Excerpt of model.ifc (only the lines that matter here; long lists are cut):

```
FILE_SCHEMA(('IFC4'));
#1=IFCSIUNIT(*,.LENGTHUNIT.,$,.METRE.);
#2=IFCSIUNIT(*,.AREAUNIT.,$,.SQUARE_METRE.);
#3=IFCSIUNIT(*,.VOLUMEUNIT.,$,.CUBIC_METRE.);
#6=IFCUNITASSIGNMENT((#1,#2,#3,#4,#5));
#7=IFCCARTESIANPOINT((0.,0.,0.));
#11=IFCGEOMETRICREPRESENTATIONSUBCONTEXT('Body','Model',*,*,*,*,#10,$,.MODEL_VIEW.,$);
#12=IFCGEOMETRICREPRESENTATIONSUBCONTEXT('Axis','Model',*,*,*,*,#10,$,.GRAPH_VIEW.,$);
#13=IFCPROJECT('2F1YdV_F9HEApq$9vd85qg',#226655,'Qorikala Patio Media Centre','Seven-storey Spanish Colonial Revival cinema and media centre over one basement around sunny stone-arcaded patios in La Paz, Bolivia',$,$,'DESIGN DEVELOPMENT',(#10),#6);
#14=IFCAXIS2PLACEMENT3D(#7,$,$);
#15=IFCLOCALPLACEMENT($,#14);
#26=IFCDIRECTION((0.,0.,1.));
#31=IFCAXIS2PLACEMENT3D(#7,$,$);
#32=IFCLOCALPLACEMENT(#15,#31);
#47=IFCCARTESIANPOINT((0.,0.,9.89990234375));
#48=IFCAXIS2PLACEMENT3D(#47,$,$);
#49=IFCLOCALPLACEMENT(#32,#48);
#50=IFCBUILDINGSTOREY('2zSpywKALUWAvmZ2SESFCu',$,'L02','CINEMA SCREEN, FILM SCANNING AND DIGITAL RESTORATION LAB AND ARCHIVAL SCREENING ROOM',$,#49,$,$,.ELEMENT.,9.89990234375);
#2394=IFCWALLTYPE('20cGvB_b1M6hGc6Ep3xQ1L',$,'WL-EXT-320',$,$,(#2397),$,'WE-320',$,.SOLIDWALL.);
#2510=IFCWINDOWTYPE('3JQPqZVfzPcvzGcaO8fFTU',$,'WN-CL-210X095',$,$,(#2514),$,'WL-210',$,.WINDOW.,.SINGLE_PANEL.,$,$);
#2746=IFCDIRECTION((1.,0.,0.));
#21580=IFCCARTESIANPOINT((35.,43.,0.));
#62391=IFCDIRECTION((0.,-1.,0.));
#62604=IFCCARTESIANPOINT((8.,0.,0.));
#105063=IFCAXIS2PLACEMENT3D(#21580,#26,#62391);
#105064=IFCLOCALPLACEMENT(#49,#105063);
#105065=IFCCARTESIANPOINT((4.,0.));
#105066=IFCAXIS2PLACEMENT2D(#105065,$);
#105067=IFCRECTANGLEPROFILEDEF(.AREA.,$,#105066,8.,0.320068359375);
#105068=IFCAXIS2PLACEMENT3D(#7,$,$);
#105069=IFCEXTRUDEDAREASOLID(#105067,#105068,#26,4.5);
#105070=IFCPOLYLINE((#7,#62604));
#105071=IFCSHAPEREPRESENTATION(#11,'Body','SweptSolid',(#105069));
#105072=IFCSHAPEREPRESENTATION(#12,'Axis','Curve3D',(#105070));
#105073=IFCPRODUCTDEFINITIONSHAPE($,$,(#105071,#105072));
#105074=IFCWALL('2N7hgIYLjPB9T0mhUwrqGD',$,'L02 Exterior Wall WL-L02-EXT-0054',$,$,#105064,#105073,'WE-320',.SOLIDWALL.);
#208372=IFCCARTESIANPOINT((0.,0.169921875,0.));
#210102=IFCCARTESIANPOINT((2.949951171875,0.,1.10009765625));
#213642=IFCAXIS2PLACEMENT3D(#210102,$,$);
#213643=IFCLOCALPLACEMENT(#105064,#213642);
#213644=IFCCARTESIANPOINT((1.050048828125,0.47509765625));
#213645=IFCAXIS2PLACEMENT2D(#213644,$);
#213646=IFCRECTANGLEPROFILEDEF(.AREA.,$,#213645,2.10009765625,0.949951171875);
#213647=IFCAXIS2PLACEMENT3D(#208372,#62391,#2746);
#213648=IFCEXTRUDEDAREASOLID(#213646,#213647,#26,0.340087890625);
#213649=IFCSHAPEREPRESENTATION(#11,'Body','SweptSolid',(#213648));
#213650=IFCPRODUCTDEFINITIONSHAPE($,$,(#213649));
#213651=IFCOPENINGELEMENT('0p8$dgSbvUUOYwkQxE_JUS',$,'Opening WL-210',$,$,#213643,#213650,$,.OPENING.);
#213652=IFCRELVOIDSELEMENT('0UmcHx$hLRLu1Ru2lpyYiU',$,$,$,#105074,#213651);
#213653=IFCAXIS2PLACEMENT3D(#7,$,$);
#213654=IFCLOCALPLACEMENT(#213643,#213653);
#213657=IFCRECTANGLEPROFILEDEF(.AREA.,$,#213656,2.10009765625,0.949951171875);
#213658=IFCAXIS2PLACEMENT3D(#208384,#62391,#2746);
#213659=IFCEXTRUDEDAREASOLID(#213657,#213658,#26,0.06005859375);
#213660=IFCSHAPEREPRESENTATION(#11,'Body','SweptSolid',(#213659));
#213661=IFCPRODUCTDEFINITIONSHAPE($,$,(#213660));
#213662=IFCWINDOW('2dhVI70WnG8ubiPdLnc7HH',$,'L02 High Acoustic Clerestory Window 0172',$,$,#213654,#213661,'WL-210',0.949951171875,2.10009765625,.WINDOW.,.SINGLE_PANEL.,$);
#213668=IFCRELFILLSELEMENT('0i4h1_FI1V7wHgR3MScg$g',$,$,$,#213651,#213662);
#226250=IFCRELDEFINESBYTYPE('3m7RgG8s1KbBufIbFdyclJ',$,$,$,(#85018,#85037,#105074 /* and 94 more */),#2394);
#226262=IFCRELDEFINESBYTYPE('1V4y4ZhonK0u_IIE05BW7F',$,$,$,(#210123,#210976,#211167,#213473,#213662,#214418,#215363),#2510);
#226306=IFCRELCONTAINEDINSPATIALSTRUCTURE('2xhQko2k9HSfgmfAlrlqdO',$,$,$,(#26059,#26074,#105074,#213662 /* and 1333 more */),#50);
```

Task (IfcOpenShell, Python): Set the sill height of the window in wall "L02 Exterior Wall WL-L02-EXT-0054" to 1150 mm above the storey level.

```python
import numpy as np
import ifcopenshell
import ifcopenshell.api.geometry
import ifcopenshell.geom
import ifcopenshell.util.element
import ifcopenshell.util.placement
import ifcopenshell.util.shape
import ifcopenshell.util.unit

model = ifcopenshell.open("model.ifc")
unit_scale = ifcopenshell.util.unit.calculate_unit_scale(model)

window = model.by_guid("2dhVI70WnG8ubiPdLnc7HH")
opening = window.FillsVoids[0].RelatingOpeningElement
storey = ifcopenshell.util.element.get_container(window, ifc_class="IfcBuildingStorey")
level = ifcopenshell.util.placement.get_local_placement(storey.ObjectPlacement)[2, 3]

# The opening's origin need not be at the sill, so measure its lowest point.
shape = ifcopenshell.geom.create_shape(ifcopenshell.geom.settings(), opening)
bottom = ifcopenshell.util.shape.get_shape_bottom_elevation(shape, shape.geometry) / unit_scale
dz = level + 1.15 - bottom

shift = np.array([0.0, 0.0, dz])
# The window is placed relative to its opening, so it follows when the opening moves.
matrix = ifcopenshell.util.placement.get_local_placement(opening.ObjectPlacement)
matrix[:3, 3] += shift
ifcopenshell.api.geometry.edit_object_placement(
    model, product=opening, matrix=matrix, is_si=False, should_transform_children=True
)

print(f"moved by {dz * unit_scale:+.3f} m")

model.write("model_updated.ifc")
```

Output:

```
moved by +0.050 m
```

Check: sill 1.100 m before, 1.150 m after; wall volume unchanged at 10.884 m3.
